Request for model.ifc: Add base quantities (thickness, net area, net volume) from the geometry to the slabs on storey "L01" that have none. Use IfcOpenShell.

First a look at what the model holds.

```python
import ifcopenshell
import ifcopenshell.util.element
import ifcopenshell.util.unit

model = ifcopenshell.open("model.ifc")
print(model.schema)
for unit_type in ("LENGTHUNIT", "AREAUNIT", "VOLUMEUNIT"):
    print(unit_type, ifcopenshell.util.unit.calculate_unit_scale(model, unit_type))
storey = next(s for s in model.by_type("IfcBuildingStorey") if s.Name == "L01")
slabs = [e for e in ifcopenshell.util.element.get_decomposition(storey) if e.is_a("IfcSlab")]
for e in sorted(slabs, key=lambda e: e.id()):
    print(e.id(), e.is_a(), e.Name, list(ifcopenshell.util.element.get_psets(e, qtos_only=True)), sep=" | ")
```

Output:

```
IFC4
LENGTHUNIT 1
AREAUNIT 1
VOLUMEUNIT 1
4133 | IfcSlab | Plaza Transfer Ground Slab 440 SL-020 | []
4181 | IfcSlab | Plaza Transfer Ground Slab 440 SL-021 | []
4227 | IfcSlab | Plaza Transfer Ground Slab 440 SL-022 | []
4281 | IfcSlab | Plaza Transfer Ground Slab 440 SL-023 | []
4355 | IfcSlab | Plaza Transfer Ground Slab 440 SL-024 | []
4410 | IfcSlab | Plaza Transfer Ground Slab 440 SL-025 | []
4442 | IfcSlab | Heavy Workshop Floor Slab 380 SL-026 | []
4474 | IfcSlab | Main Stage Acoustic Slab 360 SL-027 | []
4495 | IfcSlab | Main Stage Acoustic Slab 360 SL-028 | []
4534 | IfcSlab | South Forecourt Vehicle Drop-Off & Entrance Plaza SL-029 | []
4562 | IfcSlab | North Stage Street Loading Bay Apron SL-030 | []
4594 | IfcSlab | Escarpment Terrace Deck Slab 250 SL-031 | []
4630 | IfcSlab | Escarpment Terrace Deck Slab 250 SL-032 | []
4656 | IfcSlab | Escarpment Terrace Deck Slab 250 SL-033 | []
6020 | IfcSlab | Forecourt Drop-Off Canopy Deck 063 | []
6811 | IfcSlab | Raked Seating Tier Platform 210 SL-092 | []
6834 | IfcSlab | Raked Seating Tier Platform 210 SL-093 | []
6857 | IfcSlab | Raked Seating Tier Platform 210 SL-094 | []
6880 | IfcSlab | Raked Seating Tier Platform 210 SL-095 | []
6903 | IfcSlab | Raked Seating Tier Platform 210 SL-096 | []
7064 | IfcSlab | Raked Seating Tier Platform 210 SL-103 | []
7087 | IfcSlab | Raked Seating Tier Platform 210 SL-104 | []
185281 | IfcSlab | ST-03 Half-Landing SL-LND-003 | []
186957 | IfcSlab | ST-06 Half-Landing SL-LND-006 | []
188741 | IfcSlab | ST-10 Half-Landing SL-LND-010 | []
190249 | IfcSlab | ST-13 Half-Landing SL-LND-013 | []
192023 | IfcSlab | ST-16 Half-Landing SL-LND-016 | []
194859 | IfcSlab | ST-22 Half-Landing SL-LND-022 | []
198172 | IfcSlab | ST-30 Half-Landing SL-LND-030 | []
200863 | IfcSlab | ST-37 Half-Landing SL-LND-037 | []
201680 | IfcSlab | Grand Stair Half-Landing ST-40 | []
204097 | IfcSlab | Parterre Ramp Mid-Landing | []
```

```python
import ifcopenshell
import ifcopenshell.api.pset
import ifcopenshell.geom
import ifcopenshell.util.element
import ifcopenshell.util.shape
import ifcopenshell.util.unit

model = ifcopenshell.open("model.ifc")
unit_scale = ifcopenshell.util.unit.calculate_unit_scale(model)
area_scale = ifcopenshell.util.unit.calculate_unit_scale(model, "AREAUNIT")
volume_scale = ifcopenshell.util.unit.calculate_unit_scale(model, "VOLUMEUNIT")
settings = ifcopenshell.geom.settings()

storey = next(s for s in model.by_type("IfcBuildingStorey") if s.Name == "L01")
slabs = [e for e in ifcopenshell.util.element.get_decomposition(storey) if e.is_a("IfcSlab")]

for e in sorted(slabs, key=lambda e: e.id()):
    if ifcopenshell.util.element.get_psets(e, qtos_only=True, should_inherit=False):
        continue
    # Geometry comes back in metres, in the element's own axes.
    shape = ifcopenshell.geom.create_shape(settings, e)
    values = {
        "Width": ifcopenshell.util.shape.get_z(shape.geometry) / unit_scale,
        "NetArea": ifcopenshell.util.shape.get_footprint_area(shape.geometry) / area_scale,
        "NetVolume": ifcopenshell.util.shape.get_volume(shape.geometry) / volume_scale,
    }
    qto = ifcopenshell.api.pset.add_qto(model, product=e, name="Qto_SlabBaseQuantities")
    ifcopenshell.api.pset.edit_qto(model, qto=qto, properties=values)
    print(e.id(), {k: round(v, 3) for k, v in values.items()})

model.write("model_rev.ifc")
```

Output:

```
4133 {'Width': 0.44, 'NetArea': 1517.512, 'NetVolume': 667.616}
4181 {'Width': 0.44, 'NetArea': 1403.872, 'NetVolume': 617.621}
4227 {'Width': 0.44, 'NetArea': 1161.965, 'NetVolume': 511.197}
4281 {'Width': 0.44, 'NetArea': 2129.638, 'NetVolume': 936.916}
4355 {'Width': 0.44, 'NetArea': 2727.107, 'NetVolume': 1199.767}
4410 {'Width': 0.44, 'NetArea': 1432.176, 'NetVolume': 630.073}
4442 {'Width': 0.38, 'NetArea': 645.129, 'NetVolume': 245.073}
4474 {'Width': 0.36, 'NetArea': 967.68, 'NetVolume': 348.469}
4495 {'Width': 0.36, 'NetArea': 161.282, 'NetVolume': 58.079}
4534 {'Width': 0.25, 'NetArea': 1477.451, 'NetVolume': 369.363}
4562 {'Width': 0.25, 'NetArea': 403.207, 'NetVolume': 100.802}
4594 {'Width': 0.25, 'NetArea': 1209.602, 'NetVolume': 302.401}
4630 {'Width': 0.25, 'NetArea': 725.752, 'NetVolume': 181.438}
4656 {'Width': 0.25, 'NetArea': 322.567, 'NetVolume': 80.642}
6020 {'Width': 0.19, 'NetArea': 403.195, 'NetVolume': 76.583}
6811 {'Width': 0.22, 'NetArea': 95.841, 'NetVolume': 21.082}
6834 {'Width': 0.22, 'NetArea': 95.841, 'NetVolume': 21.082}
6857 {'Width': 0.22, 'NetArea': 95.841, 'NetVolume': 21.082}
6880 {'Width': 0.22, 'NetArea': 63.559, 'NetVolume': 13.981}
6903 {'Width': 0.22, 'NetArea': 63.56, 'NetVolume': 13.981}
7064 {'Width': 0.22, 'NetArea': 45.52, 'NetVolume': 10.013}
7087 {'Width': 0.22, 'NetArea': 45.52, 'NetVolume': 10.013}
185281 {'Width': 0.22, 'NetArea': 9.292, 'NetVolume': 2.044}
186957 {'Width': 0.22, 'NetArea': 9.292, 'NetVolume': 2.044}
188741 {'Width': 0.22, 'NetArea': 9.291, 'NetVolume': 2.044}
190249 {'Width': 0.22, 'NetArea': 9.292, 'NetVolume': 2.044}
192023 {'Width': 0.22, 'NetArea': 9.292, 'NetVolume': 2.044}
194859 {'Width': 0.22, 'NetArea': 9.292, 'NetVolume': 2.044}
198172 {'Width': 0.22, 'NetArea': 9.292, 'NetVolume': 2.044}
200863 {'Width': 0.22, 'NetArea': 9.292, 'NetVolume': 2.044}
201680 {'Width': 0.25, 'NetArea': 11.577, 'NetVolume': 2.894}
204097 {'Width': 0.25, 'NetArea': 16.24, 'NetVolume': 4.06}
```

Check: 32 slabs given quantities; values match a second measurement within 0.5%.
